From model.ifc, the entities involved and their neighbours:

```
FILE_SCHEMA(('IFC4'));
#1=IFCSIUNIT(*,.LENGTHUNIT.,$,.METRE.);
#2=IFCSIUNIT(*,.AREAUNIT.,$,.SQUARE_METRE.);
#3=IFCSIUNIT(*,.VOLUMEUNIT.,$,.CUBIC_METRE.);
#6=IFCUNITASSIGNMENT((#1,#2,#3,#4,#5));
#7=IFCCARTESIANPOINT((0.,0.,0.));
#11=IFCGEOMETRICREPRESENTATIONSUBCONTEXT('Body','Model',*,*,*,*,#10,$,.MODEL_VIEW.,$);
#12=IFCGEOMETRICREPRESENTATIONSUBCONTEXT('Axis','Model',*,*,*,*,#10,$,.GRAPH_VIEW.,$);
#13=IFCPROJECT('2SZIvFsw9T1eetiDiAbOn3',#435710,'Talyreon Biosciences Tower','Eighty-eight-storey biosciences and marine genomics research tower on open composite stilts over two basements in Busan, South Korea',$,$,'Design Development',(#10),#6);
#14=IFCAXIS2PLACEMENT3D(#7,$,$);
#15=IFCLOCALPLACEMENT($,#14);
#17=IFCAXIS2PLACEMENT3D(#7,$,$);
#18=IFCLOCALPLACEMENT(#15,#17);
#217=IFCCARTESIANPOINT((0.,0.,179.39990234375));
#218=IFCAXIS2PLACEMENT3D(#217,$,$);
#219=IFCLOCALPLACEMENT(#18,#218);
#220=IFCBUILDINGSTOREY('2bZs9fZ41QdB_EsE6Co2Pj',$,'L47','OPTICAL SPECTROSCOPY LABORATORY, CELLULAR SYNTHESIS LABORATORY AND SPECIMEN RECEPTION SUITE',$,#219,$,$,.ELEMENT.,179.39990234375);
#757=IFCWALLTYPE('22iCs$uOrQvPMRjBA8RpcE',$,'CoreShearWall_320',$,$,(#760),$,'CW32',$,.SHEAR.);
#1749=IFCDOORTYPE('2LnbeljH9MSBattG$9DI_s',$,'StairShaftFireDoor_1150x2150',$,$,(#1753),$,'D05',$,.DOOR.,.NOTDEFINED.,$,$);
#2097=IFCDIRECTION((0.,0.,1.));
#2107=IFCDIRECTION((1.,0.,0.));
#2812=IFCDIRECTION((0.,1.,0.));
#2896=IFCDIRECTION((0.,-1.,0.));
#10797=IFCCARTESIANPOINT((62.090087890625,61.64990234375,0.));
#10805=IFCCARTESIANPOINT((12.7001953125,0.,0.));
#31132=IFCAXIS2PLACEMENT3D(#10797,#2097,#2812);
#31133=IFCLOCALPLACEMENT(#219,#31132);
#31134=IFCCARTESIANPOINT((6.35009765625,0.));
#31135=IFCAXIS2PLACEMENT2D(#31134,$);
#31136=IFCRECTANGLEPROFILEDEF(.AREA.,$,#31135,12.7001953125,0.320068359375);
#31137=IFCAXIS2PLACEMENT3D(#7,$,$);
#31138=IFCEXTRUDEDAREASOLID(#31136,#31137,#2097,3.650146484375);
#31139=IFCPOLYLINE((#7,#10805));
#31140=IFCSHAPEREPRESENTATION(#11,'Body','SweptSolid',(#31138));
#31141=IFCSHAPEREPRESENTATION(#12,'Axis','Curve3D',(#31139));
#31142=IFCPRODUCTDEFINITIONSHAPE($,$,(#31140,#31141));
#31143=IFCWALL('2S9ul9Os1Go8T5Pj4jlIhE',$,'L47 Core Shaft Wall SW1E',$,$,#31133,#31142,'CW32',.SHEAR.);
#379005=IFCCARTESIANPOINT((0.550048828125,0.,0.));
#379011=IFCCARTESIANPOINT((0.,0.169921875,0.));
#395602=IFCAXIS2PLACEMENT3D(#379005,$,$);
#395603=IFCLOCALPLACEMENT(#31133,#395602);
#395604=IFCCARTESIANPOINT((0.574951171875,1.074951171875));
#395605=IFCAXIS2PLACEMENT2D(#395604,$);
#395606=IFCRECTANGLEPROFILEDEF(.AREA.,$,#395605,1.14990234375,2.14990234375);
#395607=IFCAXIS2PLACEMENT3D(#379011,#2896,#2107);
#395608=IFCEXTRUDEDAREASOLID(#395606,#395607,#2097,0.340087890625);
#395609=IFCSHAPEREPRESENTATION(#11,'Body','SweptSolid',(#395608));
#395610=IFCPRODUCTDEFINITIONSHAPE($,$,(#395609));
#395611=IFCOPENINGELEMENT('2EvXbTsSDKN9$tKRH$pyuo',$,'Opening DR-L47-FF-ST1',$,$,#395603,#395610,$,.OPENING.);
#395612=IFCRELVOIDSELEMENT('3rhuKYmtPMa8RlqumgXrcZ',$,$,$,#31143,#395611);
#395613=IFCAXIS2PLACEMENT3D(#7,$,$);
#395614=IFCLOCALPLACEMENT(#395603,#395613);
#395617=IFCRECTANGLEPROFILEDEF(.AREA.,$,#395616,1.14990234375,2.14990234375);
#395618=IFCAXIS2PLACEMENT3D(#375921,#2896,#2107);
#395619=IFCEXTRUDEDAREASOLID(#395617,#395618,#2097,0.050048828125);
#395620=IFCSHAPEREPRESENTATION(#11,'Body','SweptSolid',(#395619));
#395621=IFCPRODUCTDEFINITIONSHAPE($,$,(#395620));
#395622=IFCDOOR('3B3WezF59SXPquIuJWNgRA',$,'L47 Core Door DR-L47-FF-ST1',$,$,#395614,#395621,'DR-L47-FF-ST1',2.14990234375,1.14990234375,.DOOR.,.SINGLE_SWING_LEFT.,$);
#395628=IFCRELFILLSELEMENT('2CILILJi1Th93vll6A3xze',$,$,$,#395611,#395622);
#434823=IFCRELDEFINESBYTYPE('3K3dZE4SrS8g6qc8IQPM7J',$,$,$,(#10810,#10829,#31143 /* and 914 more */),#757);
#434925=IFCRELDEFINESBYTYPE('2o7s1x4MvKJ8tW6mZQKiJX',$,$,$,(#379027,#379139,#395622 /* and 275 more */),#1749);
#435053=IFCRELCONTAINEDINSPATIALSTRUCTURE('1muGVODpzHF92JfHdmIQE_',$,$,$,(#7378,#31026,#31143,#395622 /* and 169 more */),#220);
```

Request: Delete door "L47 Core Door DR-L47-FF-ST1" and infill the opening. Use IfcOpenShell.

```python
import ifcopenshell
import ifcopenshell.api.feature
import ifcopenshell.api.root
import ifcopenshell.geom
import ifcopenshell.util.shape

model = ifcopenshell.open("model.ifc")
settings = ifcopenshell.geom.settings()


def volume(element):
    """Net volume in cubic metres, openings subtracted."""
    shape = ifcopenshell.geom.create_shape(settings, element)
    return ifcopenshell.util.shape.get_volume(shape.geometry)


door = model.by_guid("3B3WezF59SXPquIuJWNgRA")
opening = door.FillsVoids[0].RelatingOpeningElement
wall = opening.VoidsElements[0].RelatingBuildingElement
before = volume(wall)

ifcopenshell.api.root.remove_product(model, product=door)
ifcopenshell.api.feature.remove_feature(model, feature=opening)

after = volume(wall)

print(f"wall volume {before:.3f} -> {after:.3f} m3")

model.write("model_rev.ifc")
```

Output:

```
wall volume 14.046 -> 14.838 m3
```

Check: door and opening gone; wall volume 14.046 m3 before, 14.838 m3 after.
